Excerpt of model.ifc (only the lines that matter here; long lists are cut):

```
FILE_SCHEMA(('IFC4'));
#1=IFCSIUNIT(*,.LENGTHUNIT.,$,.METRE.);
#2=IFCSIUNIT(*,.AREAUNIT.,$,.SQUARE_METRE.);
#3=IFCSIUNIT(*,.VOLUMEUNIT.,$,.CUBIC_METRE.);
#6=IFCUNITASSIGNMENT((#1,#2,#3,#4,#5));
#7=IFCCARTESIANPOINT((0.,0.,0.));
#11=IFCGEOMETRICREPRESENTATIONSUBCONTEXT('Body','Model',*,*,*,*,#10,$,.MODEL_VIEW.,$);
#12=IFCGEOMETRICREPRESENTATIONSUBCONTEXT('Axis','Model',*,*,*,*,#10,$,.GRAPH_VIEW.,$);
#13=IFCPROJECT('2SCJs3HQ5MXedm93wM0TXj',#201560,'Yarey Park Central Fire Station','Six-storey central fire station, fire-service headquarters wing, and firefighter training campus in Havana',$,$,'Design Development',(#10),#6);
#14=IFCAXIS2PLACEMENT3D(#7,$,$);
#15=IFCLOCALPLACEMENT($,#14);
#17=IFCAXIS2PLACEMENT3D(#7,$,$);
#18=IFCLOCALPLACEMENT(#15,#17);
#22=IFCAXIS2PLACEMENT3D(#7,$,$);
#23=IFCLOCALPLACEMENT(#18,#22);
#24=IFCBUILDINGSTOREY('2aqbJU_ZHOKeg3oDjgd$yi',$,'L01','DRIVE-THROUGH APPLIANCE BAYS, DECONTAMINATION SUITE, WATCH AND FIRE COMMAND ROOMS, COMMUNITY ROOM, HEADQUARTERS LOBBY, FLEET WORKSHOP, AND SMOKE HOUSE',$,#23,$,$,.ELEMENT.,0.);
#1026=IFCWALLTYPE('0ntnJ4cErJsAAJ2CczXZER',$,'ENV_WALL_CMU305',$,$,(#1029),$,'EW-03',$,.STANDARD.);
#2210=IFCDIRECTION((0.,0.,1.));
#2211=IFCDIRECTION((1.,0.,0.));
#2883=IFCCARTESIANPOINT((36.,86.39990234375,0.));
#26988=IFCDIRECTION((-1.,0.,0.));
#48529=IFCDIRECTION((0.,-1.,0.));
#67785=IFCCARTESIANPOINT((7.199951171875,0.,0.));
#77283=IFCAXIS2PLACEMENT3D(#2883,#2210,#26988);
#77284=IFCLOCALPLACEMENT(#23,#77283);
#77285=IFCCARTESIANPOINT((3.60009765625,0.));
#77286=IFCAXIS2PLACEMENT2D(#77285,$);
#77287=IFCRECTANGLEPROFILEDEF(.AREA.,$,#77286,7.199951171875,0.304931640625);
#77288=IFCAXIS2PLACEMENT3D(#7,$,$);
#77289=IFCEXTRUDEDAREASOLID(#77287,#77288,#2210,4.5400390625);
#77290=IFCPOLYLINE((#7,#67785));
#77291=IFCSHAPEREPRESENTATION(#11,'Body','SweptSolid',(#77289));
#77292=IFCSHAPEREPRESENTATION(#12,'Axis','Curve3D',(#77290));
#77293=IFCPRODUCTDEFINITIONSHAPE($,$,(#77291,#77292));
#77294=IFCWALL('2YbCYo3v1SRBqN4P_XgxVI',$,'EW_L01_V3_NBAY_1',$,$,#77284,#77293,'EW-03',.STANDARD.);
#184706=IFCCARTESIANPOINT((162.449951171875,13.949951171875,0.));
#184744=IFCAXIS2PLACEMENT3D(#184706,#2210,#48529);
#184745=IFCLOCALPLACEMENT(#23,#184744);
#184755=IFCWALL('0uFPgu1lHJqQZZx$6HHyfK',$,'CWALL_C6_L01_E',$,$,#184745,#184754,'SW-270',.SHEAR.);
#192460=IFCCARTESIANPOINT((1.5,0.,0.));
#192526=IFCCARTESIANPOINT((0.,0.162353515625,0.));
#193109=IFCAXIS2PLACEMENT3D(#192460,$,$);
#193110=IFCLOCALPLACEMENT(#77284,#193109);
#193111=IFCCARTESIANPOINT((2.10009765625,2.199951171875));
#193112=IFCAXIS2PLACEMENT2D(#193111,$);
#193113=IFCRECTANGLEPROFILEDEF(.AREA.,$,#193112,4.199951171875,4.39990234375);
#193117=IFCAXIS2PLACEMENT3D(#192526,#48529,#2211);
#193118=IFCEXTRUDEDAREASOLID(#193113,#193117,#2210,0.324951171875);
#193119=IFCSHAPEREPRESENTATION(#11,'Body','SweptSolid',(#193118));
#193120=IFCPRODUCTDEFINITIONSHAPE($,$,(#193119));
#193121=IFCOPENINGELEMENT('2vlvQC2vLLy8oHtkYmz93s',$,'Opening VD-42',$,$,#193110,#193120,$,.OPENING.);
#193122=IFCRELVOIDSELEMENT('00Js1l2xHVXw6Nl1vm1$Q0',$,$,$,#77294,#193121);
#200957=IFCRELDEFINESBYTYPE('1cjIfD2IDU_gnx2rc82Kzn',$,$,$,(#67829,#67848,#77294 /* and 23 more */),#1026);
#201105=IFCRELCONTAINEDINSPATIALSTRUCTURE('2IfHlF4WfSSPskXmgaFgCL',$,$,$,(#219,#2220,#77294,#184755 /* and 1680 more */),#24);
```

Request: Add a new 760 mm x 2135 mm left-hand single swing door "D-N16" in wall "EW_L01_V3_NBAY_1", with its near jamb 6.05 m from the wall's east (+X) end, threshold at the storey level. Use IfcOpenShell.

```python
import numpy as np
import ifcopenshell
import ifcopenshell.api.feature
import ifcopenshell.api.geometry
import ifcopenshell.api.root
import ifcopenshell.api.spatial
import ifcopenshell.geom
import ifcopenshell.util.element
import ifcopenshell.util.placement
import ifcopenshell.util.representation
import ifcopenshell.util.shape
import ifcopenshell.util.unit

model = ifcopenshell.open("model.ifc")
unit_scale = ifcopenshell.util.unit.calculate_unit_scale(model)
settings = ifcopenshell.geom.settings()


def volume(element):
    """Net volume in cubic metres, openings subtracted."""
    shape = ifcopenshell.geom.create_shape(settings, element)
    return ifcopenshell.util.shape.get_volume(shape.geometry)


wall = model.by_id(77294)
storey = ifcopenshell.util.element.get_container(wall, ifc_class="IfcBuildingStorey")
context = ifcopenshell.util.representation.get_context(model, "Model", "Body", "MODEL_VIEW")
before = volume(wall)

width, height, from_end, sill = 0.76, 2.135, 6.05, 0.0  # metres

# The wall runs along its own X axis, and the end named is its -X end.
wall_shape = ifcopenshell.geom.create_shape(settings, wall)
x, y, z = ifcopenshell.util.shape.get_vertices(wall_shape.geometry).T
start = x.min() + from_end
face, thickness = float(y.min()), float(y.max() - y.min())
wall_matrix = ifcopenshell.util.placement.get_local_placement(wall.ObjectPlacement)
level = ifcopenshell.util.placement.get_local_placement(storey.ObjectPlacement)[2, 3]


def in_wall(x, y):
    """Placement at x, y metres in the wall's axes, at sill height."""
    matrix = wall_matrix.copy()
    matrix[:, 3] = wall_matrix @ np.array([x / unit_scale, y / unit_scale, 0.0, 1.0])
    matrix[2, 3] = level + sill / unit_scale
    return matrix


# Opening: a box that overshoots both wall faces by 50 mm.
opening = ifcopenshell.api.root.create_entity(model, ifc_class="IfcOpeningElement", predefined_type="OPENING")
box = ifcopenshell.api.geometry.add_wall_representation(
    model, context=context, length=width, height=height, thickness=thickness + 0.1
)
ifcopenshell.api.geometry.assign_representation(model, product=opening, representation=box)
ifcopenshell.api.geometry.edit_object_placement(model, product=opening, matrix=in_wall(start, face - 0.05), is_si=False)
ifcopenshell.api.feature.add_feature(model, feature=opening, element=wall)

door = ifcopenshell.api.root.create_entity(model, ifc_class="IfcDoor", name="D-N16", predefined_type="DOOR")
door.OverallWidth, door.OverallHeight = width / unit_scale, height / unit_scale
door.OperationType = "SINGLE_SWING_LEFT"
body = ifcopenshell.api.geometry.add_door_representation(
    model,
    context=context,
    overall_width=door.OverallWidth,
    overall_height=door.OverallHeight,
    operation_type="SINGLE_SWING_LEFT",
    lining_properties={"LiningDepth": thickness / unit_scale, "ThresholdDepth": thickness / unit_scale},
)
ifcopenshell.api.geometry.assign_representation(model, product=door, representation=body)
ifcopenshell.api.spatial.assign_container(model, products=[door], relating_structure=storey)
ifcopenshell.api.feature.add_filling(model, opening=opening, element=door)

# The lining spans the wall, so the door starts at the wall face.
ifcopenshell.api.geometry.edit_object_placement(model, product=door, matrix=in_wall(start, face), is_si=False)

after = volume(wall)

print(f"wall volume {before:.3f} -> {after:.3f} m3")

model.write("model_v2.ifc")
```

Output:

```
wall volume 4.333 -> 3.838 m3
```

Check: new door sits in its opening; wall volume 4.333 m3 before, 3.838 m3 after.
